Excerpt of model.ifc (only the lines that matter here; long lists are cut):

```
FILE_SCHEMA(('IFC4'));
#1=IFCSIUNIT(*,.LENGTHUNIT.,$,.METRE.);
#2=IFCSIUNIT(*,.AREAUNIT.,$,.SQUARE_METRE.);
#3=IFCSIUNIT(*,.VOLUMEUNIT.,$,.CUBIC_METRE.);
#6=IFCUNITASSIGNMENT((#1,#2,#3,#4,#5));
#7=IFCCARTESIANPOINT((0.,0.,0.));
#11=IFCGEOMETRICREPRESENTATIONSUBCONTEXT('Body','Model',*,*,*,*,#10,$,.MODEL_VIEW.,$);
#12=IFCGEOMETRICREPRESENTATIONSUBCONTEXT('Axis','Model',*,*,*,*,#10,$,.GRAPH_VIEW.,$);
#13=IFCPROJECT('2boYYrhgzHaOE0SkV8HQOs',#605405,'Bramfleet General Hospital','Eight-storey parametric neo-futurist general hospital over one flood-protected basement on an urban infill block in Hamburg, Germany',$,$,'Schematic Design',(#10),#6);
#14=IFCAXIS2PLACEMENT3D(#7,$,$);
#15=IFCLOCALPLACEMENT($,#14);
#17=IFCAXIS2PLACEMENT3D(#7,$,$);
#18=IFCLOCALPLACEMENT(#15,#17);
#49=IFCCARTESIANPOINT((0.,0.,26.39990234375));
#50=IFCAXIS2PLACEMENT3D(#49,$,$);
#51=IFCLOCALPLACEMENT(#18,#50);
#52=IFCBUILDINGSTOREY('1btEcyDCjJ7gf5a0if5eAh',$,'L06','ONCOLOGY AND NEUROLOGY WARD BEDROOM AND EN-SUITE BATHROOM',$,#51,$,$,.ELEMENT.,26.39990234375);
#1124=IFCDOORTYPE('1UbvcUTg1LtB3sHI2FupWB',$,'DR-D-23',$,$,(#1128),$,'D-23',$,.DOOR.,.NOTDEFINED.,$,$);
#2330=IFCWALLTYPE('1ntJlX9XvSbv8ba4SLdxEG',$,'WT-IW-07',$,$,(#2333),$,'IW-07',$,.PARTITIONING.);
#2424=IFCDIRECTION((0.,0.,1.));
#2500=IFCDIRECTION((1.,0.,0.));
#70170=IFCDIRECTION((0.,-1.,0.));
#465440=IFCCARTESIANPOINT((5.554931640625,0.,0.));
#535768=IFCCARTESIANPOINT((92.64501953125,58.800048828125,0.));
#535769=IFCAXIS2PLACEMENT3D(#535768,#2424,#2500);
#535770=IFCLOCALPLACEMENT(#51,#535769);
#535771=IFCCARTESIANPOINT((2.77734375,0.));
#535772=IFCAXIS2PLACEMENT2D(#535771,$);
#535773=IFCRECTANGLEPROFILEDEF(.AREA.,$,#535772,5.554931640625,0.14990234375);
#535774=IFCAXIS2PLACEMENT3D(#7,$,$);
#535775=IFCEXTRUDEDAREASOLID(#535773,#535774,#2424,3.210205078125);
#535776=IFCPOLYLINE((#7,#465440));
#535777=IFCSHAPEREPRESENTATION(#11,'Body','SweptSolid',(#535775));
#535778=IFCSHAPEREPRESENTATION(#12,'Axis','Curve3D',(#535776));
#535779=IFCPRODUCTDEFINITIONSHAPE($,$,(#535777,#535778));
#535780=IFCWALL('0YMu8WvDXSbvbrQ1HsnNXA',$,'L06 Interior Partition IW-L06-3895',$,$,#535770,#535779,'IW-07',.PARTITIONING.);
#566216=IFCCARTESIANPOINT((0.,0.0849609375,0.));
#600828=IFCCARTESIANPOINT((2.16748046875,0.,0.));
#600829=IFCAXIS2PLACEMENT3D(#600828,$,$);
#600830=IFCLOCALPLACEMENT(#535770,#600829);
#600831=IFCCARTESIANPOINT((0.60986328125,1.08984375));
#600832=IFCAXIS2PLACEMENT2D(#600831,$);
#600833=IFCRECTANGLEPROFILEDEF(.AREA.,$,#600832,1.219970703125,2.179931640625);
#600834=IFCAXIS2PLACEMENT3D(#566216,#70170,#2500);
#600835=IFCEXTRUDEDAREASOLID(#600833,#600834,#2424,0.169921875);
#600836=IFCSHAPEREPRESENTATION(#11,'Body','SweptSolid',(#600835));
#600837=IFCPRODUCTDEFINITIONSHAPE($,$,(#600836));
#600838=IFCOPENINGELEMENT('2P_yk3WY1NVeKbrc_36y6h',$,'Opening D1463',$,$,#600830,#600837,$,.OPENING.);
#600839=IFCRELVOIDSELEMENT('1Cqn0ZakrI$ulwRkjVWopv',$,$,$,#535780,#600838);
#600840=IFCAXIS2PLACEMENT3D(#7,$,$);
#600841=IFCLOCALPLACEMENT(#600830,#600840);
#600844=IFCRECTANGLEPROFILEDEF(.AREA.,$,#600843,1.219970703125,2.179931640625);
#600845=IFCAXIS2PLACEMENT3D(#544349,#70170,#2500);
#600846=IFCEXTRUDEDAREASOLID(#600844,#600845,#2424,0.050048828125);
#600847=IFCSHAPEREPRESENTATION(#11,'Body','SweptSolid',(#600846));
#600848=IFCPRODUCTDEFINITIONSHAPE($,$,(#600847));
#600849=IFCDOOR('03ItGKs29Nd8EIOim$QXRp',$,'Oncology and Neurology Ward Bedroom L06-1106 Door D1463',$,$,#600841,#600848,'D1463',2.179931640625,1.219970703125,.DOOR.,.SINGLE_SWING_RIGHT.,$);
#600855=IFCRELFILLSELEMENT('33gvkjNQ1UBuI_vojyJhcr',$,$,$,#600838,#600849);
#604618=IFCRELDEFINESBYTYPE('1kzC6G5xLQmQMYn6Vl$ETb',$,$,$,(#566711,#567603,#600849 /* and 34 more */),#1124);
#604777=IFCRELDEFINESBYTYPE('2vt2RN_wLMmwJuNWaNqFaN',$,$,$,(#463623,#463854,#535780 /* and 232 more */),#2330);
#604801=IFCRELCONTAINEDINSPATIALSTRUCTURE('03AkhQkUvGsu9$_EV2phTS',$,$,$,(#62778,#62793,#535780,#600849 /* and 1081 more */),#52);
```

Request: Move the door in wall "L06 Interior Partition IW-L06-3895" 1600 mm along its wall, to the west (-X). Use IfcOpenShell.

```python
import ifcopenshell
import ifcopenshell.api.geometry
import ifcopenshell.util.placement
import ifcopenshell.util.unit

model = ifcopenshell.open("model.ifc")
unit_scale = ifcopenshell.util.unit.calculate_unit_scale(model)

door = model.by_guid("03ItGKs29Nd8EIOim$QXRp")
opening = door.FillsVoids[0].RelatingOpeningElement
wall = opening.VoidsElements[0].RelatingBuildingElement

wall_matrix = ifcopenshell.util.placement.get_local_placement(wall.ObjectPlacement)
shift = wall_matrix[:3, 0] * -1.6 / unit_scale
before = ifcopenshell.util.placement.get_local_placement(door.ObjectPlacement)[:3, 3].copy()

# The door is placed relative to its opening, so it follows when the opening moves.
matrix = ifcopenshell.util.placement.get_local_placement(opening.ObjectPlacement)
matrix[:3, 3] += shift
ifcopenshell.api.geometry.edit_object_placement(
    model, product=opening, matrix=matrix, is_si=False, should_transform_children=True
)

after = ifcopenshell.util.placement.get_local_placement(door.ObjectPlacement)[:3, 3]
print("door moved by", (after - before).round(3) + 0.0)

model.write("model_edited.ifc")
```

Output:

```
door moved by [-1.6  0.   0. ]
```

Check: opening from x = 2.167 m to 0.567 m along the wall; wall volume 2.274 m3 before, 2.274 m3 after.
